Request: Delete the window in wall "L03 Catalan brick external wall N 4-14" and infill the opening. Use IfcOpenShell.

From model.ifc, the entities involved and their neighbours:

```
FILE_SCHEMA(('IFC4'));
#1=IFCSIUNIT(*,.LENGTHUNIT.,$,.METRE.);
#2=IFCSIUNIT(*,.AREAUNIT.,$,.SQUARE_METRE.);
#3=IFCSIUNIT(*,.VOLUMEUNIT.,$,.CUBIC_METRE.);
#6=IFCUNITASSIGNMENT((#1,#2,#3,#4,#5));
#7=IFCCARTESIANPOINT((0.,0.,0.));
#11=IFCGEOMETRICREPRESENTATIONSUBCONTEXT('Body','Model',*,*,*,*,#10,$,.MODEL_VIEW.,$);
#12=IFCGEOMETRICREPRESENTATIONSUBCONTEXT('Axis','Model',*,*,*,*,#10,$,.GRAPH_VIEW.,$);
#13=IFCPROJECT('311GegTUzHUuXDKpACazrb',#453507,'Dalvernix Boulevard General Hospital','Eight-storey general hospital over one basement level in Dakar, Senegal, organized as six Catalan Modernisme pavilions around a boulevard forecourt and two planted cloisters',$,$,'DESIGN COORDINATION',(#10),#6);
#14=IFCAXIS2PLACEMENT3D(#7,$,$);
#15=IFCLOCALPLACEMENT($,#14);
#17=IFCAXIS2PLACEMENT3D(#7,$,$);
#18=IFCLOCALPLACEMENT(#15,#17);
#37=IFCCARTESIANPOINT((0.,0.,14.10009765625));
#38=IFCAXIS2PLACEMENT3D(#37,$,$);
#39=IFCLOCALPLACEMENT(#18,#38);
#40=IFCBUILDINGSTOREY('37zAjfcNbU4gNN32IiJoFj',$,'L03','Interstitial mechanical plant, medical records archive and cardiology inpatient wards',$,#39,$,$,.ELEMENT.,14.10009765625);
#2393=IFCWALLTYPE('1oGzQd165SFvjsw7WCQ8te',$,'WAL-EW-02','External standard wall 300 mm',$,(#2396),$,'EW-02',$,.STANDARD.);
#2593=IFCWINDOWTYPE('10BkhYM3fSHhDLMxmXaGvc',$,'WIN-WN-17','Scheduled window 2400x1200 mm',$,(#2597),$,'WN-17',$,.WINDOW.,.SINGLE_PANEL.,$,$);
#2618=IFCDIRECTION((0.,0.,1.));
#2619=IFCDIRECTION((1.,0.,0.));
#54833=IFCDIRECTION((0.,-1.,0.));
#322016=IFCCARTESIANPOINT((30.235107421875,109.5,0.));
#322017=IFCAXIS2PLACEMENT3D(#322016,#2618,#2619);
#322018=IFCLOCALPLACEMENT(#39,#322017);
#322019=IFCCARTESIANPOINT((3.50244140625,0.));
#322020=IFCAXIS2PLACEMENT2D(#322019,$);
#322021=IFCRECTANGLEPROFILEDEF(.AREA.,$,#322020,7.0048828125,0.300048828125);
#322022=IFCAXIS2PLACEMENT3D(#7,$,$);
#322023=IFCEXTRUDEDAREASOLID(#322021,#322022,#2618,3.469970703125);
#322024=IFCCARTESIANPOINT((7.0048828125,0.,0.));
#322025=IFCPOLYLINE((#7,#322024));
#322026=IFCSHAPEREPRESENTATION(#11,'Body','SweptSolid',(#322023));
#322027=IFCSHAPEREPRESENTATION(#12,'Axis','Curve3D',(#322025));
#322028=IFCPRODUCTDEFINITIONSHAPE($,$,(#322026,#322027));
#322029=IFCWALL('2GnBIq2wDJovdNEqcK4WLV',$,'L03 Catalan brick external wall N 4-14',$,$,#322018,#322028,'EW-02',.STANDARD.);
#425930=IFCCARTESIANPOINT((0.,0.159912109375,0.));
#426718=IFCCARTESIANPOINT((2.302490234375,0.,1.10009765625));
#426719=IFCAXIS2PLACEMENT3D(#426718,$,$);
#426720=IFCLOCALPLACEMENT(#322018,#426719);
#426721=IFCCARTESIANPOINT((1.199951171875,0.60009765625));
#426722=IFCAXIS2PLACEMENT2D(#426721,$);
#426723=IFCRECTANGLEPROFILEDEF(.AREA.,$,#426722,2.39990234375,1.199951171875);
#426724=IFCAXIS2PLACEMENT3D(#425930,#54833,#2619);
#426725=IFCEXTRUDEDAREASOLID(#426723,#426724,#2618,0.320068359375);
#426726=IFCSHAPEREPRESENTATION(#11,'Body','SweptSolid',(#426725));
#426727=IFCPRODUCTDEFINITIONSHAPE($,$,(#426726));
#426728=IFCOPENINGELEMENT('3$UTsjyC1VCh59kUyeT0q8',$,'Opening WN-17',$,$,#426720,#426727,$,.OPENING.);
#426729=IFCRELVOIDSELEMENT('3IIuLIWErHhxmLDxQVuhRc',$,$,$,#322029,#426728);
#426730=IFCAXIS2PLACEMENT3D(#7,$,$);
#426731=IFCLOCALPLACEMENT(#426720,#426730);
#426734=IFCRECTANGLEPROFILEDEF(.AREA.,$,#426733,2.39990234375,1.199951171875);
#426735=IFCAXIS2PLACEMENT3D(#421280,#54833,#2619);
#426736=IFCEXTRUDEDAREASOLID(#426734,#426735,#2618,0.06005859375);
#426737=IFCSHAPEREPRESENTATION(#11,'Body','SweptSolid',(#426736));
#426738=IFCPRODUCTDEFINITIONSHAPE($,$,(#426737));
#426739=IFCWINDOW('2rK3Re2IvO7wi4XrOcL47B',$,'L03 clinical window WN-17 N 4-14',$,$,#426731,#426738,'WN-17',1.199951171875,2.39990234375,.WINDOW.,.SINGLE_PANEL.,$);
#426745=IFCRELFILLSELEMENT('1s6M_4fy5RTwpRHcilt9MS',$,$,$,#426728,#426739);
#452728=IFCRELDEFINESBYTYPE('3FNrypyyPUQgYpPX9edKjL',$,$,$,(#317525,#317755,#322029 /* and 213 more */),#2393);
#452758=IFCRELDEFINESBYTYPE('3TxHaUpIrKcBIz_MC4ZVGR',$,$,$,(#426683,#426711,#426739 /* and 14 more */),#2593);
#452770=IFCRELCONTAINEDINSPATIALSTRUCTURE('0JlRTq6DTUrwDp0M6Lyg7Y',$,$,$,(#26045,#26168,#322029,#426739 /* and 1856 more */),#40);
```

```python
import ifcopenshell
import ifcopenshell.api.feature
import ifcopenshell.api.root
import ifcopenshell.geom
import ifcopenshell.util.shape

model = ifcopenshell.open("model.ifc")
settings = ifcopenshell.geom.settings()


def volume(element):
    """Net volume in cubic metres, openings subtracted."""
    shape = ifcopenshell.geom.create_shape(settings, element)
    return ifcopenshell.util.shape.get_volume(shape.geometry)


window = model.by_guid("2rK3Re2IvO7wi4XrOcL47B")
opening = window.FillsVoids[0].RelatingOpeningElement
wall = opening.VoidsElements[0].RelatingBuildingElement
before = volume(wall)

ifcopenshell.api.root.remove_product(model, product=window)
ifcopenshell.api.feature.remove_feature(model, feature=opening)

after = volume(wall)

print(f"wall volume {before:.3f} -> {after:.3f} m3")

model.write("model_v2.ifc")
```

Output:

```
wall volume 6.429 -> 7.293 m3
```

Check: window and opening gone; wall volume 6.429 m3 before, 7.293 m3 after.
